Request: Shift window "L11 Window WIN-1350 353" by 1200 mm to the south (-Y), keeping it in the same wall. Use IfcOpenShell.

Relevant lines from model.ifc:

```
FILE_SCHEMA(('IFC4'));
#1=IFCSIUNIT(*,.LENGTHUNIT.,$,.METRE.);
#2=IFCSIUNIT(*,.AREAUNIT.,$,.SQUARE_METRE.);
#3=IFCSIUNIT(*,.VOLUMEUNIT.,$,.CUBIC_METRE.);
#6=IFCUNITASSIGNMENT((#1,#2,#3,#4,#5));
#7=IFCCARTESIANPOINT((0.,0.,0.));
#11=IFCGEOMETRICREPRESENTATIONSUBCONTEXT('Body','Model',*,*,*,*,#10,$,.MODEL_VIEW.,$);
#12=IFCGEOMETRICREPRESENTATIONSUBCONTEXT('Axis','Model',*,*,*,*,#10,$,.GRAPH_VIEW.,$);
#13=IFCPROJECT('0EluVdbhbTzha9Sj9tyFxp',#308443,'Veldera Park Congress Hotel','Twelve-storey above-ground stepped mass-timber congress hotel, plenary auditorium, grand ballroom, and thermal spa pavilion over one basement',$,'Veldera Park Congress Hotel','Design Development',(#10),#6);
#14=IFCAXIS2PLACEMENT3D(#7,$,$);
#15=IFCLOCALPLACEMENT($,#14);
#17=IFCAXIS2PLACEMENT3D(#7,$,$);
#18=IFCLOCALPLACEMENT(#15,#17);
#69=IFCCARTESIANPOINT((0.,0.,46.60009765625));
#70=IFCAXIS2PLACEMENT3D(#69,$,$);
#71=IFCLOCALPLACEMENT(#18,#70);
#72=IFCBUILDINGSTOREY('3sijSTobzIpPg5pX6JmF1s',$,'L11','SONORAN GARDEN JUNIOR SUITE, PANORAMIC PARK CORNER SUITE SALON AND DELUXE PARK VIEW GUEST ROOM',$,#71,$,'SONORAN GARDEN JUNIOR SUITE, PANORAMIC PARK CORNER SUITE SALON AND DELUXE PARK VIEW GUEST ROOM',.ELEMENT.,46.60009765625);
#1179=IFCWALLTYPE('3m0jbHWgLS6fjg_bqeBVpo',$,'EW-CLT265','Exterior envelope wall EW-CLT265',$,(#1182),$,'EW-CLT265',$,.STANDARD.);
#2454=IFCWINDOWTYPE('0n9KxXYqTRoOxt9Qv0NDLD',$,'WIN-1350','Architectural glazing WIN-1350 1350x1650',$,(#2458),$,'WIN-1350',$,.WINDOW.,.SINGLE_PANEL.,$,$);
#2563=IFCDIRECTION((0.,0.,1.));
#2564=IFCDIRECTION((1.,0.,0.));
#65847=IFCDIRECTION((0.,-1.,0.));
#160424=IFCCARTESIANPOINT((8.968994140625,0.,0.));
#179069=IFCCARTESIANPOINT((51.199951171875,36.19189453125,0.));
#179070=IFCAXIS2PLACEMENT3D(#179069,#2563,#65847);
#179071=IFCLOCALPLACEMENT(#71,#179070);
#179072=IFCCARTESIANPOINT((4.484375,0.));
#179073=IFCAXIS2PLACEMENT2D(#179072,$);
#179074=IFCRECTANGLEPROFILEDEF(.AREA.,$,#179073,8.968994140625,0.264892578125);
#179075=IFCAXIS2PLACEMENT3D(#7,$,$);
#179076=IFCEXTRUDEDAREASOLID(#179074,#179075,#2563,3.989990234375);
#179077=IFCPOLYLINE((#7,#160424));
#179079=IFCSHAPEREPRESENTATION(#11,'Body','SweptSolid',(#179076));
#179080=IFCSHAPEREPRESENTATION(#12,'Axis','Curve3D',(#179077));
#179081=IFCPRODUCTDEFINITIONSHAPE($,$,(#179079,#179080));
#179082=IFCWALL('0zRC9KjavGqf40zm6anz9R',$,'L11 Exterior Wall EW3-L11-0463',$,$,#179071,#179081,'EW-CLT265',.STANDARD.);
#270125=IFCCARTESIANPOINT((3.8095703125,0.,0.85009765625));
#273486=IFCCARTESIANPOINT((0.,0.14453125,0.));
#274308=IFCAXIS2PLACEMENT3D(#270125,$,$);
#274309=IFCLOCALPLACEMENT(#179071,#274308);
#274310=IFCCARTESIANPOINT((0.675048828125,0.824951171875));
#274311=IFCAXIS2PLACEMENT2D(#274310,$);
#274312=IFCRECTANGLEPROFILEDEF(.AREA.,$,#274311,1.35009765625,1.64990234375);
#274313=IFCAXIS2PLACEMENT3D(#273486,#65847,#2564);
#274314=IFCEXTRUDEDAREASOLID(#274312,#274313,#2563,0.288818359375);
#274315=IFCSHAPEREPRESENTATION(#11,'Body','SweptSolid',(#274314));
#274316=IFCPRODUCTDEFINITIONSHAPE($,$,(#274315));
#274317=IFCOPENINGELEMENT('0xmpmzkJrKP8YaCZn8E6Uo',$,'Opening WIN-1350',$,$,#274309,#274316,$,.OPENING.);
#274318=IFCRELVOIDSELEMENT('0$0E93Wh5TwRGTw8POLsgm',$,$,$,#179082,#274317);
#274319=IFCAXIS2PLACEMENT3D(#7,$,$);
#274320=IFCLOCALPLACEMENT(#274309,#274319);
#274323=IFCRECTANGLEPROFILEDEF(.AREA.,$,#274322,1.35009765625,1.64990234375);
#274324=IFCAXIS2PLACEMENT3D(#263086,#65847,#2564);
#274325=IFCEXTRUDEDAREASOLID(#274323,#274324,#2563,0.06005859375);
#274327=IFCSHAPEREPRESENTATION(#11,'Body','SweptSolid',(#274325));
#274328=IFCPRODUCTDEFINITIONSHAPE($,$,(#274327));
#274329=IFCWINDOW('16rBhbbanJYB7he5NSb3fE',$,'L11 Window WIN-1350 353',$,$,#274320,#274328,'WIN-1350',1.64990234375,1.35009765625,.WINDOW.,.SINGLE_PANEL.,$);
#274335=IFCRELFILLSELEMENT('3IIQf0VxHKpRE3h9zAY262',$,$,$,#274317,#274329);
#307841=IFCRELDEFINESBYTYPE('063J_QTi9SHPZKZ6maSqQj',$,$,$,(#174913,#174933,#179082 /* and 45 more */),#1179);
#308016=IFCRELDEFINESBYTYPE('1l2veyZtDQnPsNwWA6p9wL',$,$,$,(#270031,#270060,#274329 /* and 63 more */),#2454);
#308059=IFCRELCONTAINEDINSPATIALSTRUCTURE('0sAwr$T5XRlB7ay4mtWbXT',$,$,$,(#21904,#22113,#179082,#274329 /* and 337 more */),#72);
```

```python
import ifcopenshell
import ifcopenshell.api.geometry
import ifcopenshell.util.placement
import ifcopenshell.util.unit

model = ifcopenshell.open("model.ifc")
unit_scale = ifcopenshell.util.unit.calculate_unit_scale(model)

window = model.by_guid("16rBhbbanJYB7he5NSb3fE")
opening = window.FillsVoids[0].RelatingOpeningElement
wall = opening.VoidsElements[0].RelatingBuildingElement

wall_matrix = ifcopenshell.util.placement.get_local_placement(wall.ObjectPlacement)
shift = wall_matrix[:3, 0] * 1.2 / unit_scale
before = ifcopenshell.util.placement.get_local_placement(window.ObjectPlacement)[:3, 3].copy()

# The window is placed relative to its opening, so it follows when the opening moves.
matrix = ifcopenshell.util.placement.get_local_placement(opening.ObjectPlacement)
matrix[:3, 3] += shift
ifcopenshell.api.geometry.edit_object_placement(
    model, product=opening, matrix=matrix, is_si=False, should_transform_children=True
)

after = ifcopenshell.util.placement.get_local_placement(window.ObjectPlacement)[:3, 3]
print("window moved by", (after - before).round(3) + 0.0)

model.write("model_edited.ifc")
```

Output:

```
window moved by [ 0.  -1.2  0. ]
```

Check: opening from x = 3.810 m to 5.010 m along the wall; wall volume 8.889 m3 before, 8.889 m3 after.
